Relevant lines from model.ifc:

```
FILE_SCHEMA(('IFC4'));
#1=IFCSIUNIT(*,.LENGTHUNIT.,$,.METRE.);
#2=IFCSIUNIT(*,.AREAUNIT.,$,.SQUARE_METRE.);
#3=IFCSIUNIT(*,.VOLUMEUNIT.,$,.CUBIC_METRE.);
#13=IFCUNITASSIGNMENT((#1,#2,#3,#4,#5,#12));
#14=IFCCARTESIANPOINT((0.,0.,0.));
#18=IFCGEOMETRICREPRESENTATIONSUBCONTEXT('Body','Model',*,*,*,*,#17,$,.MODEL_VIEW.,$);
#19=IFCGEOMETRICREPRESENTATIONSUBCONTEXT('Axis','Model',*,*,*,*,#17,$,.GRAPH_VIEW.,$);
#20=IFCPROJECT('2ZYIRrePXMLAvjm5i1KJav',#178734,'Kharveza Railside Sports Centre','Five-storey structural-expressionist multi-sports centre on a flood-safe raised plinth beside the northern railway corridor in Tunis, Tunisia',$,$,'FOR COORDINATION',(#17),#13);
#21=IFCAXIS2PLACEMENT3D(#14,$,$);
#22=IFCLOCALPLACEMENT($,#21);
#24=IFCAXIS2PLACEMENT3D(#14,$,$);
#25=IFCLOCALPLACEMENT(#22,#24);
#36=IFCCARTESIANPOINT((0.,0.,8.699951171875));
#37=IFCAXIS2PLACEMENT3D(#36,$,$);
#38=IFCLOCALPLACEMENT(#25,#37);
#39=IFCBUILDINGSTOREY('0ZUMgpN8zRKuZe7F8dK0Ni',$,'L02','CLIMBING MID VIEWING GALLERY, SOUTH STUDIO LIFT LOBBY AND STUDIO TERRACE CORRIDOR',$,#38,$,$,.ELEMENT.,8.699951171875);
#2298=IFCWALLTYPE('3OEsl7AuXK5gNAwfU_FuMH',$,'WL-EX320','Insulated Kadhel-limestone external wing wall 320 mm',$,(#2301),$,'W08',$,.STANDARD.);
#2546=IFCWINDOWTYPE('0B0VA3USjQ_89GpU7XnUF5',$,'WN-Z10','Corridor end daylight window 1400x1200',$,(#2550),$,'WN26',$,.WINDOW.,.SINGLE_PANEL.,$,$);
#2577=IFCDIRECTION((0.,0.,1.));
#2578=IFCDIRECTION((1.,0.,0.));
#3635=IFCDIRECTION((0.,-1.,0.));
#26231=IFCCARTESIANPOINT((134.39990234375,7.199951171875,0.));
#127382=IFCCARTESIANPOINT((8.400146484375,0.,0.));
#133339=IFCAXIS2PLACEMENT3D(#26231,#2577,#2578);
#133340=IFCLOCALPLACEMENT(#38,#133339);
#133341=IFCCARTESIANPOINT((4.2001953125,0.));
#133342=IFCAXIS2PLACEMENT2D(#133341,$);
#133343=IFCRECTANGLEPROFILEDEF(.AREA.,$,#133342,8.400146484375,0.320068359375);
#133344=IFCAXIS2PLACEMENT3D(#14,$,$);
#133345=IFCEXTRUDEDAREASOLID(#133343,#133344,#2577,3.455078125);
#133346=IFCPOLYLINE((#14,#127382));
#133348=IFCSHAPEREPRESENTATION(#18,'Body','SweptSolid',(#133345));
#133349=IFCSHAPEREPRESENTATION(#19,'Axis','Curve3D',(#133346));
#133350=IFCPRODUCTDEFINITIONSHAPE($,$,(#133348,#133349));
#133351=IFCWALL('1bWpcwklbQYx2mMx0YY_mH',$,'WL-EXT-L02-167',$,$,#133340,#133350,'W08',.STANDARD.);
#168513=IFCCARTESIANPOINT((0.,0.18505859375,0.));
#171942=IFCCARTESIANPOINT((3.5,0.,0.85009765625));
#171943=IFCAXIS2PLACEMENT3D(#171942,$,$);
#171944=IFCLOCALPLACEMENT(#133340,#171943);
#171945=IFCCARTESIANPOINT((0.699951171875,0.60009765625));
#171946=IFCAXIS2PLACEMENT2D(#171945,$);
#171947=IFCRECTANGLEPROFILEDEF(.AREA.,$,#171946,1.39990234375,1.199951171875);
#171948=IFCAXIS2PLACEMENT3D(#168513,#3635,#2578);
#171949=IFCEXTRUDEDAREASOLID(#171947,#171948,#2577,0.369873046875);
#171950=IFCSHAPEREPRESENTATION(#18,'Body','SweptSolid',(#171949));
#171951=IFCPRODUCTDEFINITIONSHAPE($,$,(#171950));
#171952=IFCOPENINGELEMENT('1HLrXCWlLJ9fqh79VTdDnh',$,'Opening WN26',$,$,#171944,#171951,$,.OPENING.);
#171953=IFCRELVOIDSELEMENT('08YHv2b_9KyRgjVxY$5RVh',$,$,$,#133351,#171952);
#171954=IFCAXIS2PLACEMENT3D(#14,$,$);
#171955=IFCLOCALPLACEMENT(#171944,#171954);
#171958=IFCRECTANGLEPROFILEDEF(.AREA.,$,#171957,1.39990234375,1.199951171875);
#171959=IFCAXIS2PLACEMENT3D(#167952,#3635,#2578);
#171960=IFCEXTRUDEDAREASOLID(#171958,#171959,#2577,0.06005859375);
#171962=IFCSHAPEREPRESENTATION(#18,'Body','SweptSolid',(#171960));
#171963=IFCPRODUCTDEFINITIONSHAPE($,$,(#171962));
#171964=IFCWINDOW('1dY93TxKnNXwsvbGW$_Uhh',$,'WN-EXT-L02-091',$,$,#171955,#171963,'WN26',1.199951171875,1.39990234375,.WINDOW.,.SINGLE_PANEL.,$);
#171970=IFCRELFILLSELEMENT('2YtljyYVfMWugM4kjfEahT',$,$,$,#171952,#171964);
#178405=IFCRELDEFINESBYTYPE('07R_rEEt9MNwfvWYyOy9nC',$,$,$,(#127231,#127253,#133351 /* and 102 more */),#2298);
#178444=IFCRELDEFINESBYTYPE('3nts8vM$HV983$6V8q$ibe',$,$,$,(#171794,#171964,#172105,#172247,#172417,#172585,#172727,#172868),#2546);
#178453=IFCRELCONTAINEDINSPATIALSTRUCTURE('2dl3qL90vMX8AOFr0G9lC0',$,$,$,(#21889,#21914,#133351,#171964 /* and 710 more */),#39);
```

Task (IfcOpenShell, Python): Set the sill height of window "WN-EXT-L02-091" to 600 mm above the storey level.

```python
import numpy as np
import ifcopenshell
import ifcopenshell.api.geometry
import ifcopenshell.geom
import ifcopenshell.util.element
import ifcopenshell.util.placement
import ifcopenshell.util.shape
import ifcopenshell.util.unit

model = ifcopenshell.open("model.ifc")
unit_scale = ifcopenshell.util.unit.calculate_unit_scale(model)

window = model.by_guid("1dY93TxKnNXwsvbGW$_Uhh")
opening = window.FillsVoids[0].RelatingOpeningElement
storey = ifcopenshell.util.element.get_container(window, ifc_class="IfcBuildingStorey")
level = ifcopenshell.util.placement.get_local_placement(storey.ObjectPlacement)[2, 3]

# The opening's origin need not be at the sill, so measure its lowest point.
shape = ifcopenshell.geom.create_shape(ifcopenshell.geom.settings(), opening)
bottom = ifcopenshell.util.shape.get_shape_bottom_elevation(shape, shape.geometry) / unit_scale
dz = level + 0.6 / unit_scale - bottom

shift = np.array([0.0, 0.0, dz])
# The window is placed relative to its opening, so it follows when the opening moves.
matrix = ifcopenshell.util.placement.get_local_placement(opening.ObjectPlacement)
matrix[:3, 3] += shift
ifcopenshell.api.geometry.edit_object_placement(
    model, product=opening, matrix=matrix, is_si=False, should_transform_children=True
)

print(f"moved by {dz * unit_scale:+.3f} m")

model.write("model-out.ifc")
```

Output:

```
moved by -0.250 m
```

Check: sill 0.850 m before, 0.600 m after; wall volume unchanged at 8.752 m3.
